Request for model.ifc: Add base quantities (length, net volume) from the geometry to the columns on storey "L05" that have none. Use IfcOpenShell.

First a look at what the model holds.

```python
import ifcopenshell
import ifcopenshell.util.element
import ifcopenshell.util.unit

model = ifcopenshell.open("model.ifc")
print(model.schema)
for unit_type in ("LENGTHUNIT", "AREAUNIT", "VOLUMEUNIT"):
    print(unit_type, ifcopenshell.util.unit.calculate_unit_scale(model, unit_type))
storey = next(s for s in model.by_type("IfcBuildingStorey") if s.Name == "L05")
columns = [e for e in ifcopenshell.util.element.get_decomposition(storey) if e.is_a("IfcColumn")]
for e in sorted(columns, key=lambda e: e.id()):
    print(e.id(), e.is_a(), e.Name, list(ifcopenshell.util.element.get_psets(e, qtos_only=True)), sep=" | ")
```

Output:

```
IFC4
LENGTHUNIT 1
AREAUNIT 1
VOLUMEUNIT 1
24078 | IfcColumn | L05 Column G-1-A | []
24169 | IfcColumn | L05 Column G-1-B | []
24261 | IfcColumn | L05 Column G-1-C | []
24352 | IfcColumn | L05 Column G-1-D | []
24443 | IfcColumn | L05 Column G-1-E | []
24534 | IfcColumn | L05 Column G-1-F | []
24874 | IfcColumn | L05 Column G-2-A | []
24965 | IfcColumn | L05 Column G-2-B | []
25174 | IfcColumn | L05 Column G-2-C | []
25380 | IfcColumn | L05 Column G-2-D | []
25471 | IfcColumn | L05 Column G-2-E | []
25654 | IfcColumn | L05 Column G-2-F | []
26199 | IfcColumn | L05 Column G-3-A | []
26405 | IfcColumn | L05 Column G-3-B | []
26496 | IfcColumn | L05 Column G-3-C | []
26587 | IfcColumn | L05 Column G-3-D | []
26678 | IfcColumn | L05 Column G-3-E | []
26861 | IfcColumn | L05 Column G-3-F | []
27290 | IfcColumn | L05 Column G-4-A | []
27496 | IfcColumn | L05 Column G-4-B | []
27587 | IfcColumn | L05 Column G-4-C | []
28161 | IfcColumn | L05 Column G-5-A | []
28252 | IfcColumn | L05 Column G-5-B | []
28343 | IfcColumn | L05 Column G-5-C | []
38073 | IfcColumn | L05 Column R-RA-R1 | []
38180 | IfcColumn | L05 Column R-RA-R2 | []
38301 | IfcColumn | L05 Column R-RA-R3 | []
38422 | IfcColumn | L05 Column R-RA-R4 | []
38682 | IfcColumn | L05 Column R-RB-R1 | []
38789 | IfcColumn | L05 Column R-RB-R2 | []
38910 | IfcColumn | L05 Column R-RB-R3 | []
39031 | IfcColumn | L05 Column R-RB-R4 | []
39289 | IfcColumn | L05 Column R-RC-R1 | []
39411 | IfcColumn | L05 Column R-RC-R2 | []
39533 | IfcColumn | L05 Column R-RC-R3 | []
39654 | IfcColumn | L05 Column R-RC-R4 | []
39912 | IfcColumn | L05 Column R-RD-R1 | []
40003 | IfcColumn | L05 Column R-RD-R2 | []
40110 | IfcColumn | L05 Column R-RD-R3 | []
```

```python
import ifcopenshell
import ifcopenshell.api.pset
import ifcopenshell.geom
import ifcopenshell.util.element
import ifcopenshell.util.shape
import ifcopenshell.util.unit

model = ifcopenshell.open("model.ifc")
unit_scale = ifcopenshell.util.unit.calculate_unit_scale(model)
volume_scale = ifcopenshell.util.unit.calculate_unit_scale(model, "VOLUMEUNIT")
settings = ifcopenshell.geom.settings()

storey = next(s for s in model.by_type("IfcBuildingStorey") if s.Name == "L05")
columns = [e for e in ifcopenshell.util.element.get_decomposition(storey) if e.is_a("IfcColumn")]

for e in sorted(columns, key=lambda e: e.id()):
    if ifcopenshell.util.element.get_psets(e, qtos_only=True, should_inherit=False):
        continue
    # Geometry comes back in metres, in the element's own axes.
    shape = ifcopenshell.geom.create_shape(settings, e)
    values = {
        "Length": ifcopenshell.util.shape.get_z(shape.geometry) / unit_scale,
        "NetVolume": ifcopenshell.util.shape.get_volume(shape.geometry) / volume_scale,
    }
    qto = ifcopenshell.api.pset.add_qto(model, product=e, name="Qto_ColumnBaseQuantities")
    ifcopenshell.api.pset.edit_qto(model, qto=qto, properties=values)
    print(e.id(), {k: round(v, 3) for k, v in values.items()})

model.write("model-out.ifc")
```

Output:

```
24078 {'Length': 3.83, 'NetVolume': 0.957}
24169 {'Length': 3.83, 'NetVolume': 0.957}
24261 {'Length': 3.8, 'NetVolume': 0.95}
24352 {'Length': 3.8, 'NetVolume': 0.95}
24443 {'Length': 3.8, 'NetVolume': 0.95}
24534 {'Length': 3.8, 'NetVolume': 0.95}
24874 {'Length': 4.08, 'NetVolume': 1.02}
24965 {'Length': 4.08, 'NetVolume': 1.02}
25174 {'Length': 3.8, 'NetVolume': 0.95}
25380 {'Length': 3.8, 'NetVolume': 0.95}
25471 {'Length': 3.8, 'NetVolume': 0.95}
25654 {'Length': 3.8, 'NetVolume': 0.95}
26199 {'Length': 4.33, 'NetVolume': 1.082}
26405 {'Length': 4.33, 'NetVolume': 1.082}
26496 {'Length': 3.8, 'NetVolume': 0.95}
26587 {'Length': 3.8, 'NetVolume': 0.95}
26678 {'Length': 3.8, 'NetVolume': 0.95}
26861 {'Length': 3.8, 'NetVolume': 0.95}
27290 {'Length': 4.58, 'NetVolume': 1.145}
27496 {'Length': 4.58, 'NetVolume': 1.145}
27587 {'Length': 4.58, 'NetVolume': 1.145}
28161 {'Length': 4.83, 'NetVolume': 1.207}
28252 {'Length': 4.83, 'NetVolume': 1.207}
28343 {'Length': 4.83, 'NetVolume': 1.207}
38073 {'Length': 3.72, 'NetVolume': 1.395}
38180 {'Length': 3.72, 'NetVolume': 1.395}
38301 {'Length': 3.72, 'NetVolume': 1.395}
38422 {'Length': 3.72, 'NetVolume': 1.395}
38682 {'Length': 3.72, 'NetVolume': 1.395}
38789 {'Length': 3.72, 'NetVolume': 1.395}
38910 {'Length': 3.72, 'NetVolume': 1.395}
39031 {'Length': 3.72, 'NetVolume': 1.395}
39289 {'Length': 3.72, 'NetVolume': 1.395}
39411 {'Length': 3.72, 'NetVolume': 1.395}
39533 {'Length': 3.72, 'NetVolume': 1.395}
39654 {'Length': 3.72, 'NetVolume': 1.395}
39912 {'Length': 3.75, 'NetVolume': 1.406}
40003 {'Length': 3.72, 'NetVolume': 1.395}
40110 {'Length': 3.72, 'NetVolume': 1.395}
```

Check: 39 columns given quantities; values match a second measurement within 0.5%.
